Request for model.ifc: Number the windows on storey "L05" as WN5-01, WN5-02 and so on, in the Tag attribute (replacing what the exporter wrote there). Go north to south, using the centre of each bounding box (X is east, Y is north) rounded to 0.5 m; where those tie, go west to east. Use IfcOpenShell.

First a look at what the model holds.

```python
import ifcopenshell
import ifcopenshell.util.element
import ifcopenshell.util.placement

model = ifcopenshell.open("model.ifc")
print(model.schema)
storey = next(s for s in model.by_type("IfcBuildingStorey") if s.Name == "L05")
windows = [e for e in ifcopenshell.util.element.get_decomposition(storey) if e.is_a("IfcWindow")]
for e in sorted(windows, key=lambda e: e.id()):
    origin = ifcopenshell.util.placement.get_local_placement(e.ObjectPlacement)[:3, 3]
    print(e.id(), e.Tag, e.Name, origin.round(2) + 0.0, sep=" | ")
```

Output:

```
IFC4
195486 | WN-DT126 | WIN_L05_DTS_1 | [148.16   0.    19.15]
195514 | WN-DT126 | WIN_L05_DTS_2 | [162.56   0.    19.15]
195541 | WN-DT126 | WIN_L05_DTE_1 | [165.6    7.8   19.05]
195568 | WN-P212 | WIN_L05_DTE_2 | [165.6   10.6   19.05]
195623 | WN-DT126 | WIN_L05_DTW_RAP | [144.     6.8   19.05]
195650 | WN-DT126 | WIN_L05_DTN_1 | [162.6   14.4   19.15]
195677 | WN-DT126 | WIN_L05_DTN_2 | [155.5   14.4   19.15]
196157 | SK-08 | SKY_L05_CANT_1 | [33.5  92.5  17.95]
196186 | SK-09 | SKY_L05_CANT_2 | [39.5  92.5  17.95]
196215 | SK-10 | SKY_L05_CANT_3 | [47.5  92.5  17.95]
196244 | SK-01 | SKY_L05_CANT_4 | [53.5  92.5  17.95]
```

```python
import ifcopenshell
import ifcopenshell.geom
import ifcopenshell.util.element
import ifcopenshell.util.shape

model = ifcopenshell.open("model.ifc")
settings = ifcopenshell.geom.settings()
settings.set("use-world-coords", True)


def centre(element):
    shape = ifcopenshell.geom.create_shape(settings, element)
    return ifcopenshell.util.shape.get_bbox_centroid(shape.geometry)


storey = next(s for s in model.by_type("IfcBuildingStorey") if s.Name == "L05")
windows = [e for e in ifcopenshell.util.element.get_decomposition(storey) if e.is_a("IfcWindow")]

# Insertion points can sit at a corner or the storey origin, so sort by the geometry (in metres).
centres = {e: centre(e) for e in windows}
windows.sort(key=lambda e: (-round(centres[e][1] / 0.5), centres[e][0]))

for i, e in enumerate(windows, start=1):
    number = f"WN5-{i:02d}"
    e.Tag = number
    print(e.id(), number)

model.write("model_updated.ifc")
```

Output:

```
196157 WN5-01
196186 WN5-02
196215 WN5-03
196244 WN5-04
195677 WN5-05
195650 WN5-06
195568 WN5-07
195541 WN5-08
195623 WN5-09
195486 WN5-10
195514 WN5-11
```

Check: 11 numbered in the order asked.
